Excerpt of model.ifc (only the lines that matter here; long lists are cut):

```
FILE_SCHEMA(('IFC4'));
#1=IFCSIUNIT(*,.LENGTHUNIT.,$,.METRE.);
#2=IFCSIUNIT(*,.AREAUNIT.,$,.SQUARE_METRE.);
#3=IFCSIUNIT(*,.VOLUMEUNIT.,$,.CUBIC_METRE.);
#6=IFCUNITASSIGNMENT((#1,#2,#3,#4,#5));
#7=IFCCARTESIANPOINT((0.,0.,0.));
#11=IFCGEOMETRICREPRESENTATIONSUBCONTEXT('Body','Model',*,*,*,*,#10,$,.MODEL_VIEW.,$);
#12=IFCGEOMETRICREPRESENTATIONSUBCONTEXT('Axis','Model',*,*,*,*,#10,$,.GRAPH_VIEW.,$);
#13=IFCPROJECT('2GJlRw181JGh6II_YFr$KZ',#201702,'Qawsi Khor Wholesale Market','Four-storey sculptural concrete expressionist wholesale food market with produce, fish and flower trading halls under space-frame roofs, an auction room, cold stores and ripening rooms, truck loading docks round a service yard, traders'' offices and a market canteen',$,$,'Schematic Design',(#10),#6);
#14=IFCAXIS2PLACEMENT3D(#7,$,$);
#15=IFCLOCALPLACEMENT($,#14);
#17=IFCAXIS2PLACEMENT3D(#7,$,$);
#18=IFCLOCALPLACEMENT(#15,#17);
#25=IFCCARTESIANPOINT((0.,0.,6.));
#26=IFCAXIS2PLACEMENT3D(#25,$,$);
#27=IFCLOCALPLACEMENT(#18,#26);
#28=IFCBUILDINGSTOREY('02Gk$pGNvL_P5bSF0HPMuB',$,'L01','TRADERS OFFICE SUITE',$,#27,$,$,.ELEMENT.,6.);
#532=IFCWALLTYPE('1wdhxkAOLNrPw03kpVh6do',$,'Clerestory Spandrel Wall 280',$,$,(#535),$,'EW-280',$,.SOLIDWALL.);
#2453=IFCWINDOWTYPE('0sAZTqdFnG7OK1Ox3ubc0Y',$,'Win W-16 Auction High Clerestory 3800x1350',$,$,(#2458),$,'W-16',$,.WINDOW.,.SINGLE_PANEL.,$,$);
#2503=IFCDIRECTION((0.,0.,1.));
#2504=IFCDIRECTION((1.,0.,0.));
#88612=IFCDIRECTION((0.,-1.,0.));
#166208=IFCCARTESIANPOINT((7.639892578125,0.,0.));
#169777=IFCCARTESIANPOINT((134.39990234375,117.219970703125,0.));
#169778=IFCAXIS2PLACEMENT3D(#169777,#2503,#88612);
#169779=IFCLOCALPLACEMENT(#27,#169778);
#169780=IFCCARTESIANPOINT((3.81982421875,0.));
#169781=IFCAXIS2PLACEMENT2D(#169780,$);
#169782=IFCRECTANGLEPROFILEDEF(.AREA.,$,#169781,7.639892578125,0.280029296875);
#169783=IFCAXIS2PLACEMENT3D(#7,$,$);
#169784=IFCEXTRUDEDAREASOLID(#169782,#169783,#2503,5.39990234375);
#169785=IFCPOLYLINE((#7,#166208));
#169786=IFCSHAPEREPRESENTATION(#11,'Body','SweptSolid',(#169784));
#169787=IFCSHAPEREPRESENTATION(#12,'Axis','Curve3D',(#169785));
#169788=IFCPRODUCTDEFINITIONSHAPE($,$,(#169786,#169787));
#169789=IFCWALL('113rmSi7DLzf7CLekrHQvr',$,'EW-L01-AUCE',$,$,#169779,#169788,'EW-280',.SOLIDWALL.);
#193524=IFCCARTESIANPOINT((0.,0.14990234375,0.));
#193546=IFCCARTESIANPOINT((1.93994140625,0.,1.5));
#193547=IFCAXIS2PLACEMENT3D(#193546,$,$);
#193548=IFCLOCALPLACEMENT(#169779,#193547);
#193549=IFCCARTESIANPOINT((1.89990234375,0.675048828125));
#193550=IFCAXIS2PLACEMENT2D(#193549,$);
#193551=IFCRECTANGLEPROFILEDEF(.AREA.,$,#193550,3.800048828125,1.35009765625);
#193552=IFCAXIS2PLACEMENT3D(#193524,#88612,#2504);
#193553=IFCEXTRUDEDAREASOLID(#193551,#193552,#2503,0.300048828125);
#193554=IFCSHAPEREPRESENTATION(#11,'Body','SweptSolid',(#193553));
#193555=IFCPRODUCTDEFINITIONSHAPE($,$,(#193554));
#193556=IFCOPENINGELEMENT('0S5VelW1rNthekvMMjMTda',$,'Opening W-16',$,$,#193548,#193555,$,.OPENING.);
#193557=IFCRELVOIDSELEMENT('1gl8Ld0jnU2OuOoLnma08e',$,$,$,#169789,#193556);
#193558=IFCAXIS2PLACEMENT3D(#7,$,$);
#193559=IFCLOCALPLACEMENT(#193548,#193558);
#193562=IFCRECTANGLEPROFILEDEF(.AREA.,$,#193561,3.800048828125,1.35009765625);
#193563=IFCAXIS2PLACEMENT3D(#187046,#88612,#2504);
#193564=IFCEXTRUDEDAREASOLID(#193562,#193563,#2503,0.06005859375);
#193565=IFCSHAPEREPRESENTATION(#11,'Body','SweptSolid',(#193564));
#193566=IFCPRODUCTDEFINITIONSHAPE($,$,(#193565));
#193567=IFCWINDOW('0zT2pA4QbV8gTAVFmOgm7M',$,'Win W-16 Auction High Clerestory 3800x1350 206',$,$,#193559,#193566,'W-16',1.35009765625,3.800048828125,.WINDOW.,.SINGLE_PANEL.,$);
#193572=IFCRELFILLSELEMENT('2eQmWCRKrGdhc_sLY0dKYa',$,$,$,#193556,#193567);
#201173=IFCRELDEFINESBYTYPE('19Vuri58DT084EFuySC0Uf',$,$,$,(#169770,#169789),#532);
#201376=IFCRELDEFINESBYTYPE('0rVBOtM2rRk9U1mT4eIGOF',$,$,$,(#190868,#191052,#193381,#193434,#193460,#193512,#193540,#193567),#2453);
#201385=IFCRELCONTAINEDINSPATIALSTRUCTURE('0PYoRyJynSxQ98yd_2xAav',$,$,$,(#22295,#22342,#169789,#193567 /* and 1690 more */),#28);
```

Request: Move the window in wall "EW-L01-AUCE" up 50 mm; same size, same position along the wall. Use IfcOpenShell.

```python
import numpy as np
import ifcopenshell
import ifcopenshell.api.geometry
import ifcopenshell.util.placement
import ifcopenshell.util.unit

model = ifcopenshell.open("model.ifc")
unit_scale = ifcopenshell.util.unit.calculate_unit_scale(model)

window = model.by_id(193567)
opening = window.FillsVoids[0].RelatingOpeningElement
dz = 0.05

shift = np.array([0.0, 0.0, dz])
# The window is placed relative to its opening, so it follows when the opening moves.
matrix = ifcopenshell.util.placement.get_local_placement(opening.ObjectPlacement)
matrix[:3, 3] += shift
ifcopenshell.api.geometry.edit_object_placement(
    model, product=opening, matrix=matrix, is_si=False, should_transform_children=True
)

print(f"moved by {dz * unit_scale:+.3f} m")

model.write("model-out.ifc")
```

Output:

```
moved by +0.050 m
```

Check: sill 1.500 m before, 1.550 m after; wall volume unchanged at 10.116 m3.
